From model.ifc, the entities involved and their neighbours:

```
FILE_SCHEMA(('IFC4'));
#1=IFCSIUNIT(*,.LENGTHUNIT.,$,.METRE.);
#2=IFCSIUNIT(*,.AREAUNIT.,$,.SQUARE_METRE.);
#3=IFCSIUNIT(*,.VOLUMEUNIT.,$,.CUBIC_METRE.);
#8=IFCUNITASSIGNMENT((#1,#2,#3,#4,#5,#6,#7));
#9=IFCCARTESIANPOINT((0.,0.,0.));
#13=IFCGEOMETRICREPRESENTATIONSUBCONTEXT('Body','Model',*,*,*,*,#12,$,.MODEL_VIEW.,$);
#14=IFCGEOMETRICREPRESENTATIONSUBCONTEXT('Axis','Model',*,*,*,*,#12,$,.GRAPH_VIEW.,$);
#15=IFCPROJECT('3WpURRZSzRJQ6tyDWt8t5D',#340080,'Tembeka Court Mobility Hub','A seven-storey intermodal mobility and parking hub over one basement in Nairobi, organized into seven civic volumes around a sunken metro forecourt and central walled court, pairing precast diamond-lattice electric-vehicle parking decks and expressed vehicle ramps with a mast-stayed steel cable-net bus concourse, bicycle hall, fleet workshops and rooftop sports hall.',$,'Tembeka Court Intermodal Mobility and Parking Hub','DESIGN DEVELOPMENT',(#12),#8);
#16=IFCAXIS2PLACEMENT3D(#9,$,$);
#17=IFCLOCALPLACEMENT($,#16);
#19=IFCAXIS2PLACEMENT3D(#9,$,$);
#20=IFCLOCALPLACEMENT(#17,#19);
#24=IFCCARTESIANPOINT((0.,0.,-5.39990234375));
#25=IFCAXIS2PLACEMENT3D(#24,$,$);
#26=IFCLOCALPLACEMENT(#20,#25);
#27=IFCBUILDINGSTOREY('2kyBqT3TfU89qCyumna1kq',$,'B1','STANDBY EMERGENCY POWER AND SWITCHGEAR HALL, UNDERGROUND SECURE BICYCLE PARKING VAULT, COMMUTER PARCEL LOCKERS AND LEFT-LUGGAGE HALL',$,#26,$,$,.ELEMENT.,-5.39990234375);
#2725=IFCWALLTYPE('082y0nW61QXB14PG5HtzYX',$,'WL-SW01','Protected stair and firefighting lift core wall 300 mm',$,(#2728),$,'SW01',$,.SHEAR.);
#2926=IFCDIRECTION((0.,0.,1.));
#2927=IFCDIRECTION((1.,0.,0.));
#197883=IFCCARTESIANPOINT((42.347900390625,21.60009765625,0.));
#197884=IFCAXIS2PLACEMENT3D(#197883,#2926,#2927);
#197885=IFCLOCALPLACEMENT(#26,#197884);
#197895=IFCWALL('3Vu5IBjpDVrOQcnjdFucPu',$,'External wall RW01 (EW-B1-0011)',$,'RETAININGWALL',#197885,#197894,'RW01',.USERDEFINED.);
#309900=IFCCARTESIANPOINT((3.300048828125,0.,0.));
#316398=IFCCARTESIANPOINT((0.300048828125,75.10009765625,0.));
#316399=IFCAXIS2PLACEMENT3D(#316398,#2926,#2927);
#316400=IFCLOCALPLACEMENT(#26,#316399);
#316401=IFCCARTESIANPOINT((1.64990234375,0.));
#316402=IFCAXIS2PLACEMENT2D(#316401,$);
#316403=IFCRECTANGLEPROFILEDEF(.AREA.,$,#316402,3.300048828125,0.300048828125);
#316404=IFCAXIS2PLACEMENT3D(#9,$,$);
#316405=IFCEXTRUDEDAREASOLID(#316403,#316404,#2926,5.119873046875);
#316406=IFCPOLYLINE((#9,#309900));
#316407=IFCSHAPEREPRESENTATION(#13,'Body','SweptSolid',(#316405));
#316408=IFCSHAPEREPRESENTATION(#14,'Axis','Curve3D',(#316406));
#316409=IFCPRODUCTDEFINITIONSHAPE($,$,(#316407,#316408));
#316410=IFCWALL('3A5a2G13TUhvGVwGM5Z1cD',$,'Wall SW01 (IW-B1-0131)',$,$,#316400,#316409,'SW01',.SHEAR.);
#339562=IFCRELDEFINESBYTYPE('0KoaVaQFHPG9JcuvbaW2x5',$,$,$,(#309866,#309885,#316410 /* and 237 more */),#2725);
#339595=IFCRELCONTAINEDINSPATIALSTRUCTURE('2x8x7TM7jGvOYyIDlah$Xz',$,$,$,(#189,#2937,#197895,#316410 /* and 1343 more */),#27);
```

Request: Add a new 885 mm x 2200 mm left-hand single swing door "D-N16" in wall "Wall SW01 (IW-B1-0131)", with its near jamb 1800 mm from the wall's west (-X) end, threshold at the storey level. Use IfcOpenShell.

```python
import numpy as np
import ifcopenshell
import ifcopenshell.api.feature
import ifcopenshell.api.geometry
import ifcopenshell.api.root
import ifcopenshell.api.spatial
import ifcopenshell.geom
import ifcopenshell.util.element
import ifcopenshell.util.placement
import ifcopenshell.util.representation
import ifcopenshell.util.shape
import ifcopenshell.util.unit

model = ifcopenshell.open("model.ifc")
unit_scale = ifcopenshell.util.unit.calculate_unit_scale(model)
settings = ifcopenshell.geom.settings()


def volume(element):
    """Net volume in cubic metres, openings subtracted."""
    shape = ifcopenshell.geom.create_shape(settings, element)
    return ifcopenshell.util.shape.get_volume(shape.geometry)


wall = model.by_guid("3A5a2G13TUhvGVwGM5Z1cD")
storey = ifcopenshell.util.element.get_container(wall, ifc_class="IfcBuildingStorey")
context = ifcopenshell.util.representation.get_context(model, "Model", "Body", "MODEL_VIEW")
before = volume(wall)

width, height, from_end, sill = 0.885, 2.2, 1.8, 0.0  # metres

# The wall runs along its own X axis, and the end named is its -X end.
wall_shape = ifcopenshell.geom.create_shape(settings, wall)
x, y, z = ifcopenshell.util.shape.get_vertices(wall_shape.geometry).T
start = x.min() + from_end
face, thickness = float(y.min()), float(y.max() - y.min())
wall_matrix = ifcopenshell.util.placement.get_local_placement(wall.ObjectPlacement)
level = ifcopenshell.util.placement.get_local_placement(storey.ObjectPlacement)[2, 3]


def in_wall(x, y):
    """Placement at x, y metres in the wall's axes, at sill height."""
    matrix = wall_matrix.copy()
    matrix[:, 3] = wall_matrix @ np.array([x / unit_scale, y / unit_scale, 0.0, 1.0])
    matrix[2, 3] = level + sill / unit_scale
    return matrix


# Opening: a box that overshoots both wall faces by 50 mm.
opening = ifcopenshell.api.root.create_entity(model, ifc_class="IfcOpeningElement", predefined_type="OPENING")
box = ifcopenshell.api.geometry.add_wall_representation(
    model, context=context, length=width, height=height, thickness=thickness + 0.1
)
ifcopenshell.api.geometry.assign_representation(model, product=opening, representation=box)
ifcopenshell.api.geometry.edit_object_placement(model, product=opening, matrix=in_wall(start, face - 0.05), is_si=False)
ifcopenshell.api.feature.add_feature(model, feature=opening, element=wall)

door = ifcopenshell.api.root.create_entity(model, ifc_class="IfcDoor", name="D-N16", predefined_type="DOOR")
door.OverallWidth, door.OverallHeight = width / unit_scale, height / unit_scale
door.OperationType = "SINGLE_SWING_LEFT"
body = ifcopenshell.api.geometry.add_door_representation(
    model,
    context=context,
    overall_width=door.OverallWidth,
    overall_height=door.OverallHeight,
    operation_type="SINGLE_SWING_LEFT",
    lining_properties={"LiningDepth": thickness / unit_scale, "ThresholdDepth": thickness / unit_scale},
)
ifcopenshell.api.geometry.assign_representation(model, product=door, representation=body)
ifcopenshell.api.spatial.assign_container(model, products=[door], relating_structure=storey)
ifcopenshell.api.feature.add_filling(model, opening=opening, element=door)

# The lining spans the wall, so the door starts at the wall face.
ifcopenshell.api.geometry.edit_object_placement(model, product=door, matrix=in_wall(start, face), is_si=False)

after = volume(wall)

print(f"wall volume {before:.3f} -> {after:.3f} m3")

model.write("model_updated.ifc")
```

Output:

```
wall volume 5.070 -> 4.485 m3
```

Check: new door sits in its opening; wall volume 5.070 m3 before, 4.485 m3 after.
